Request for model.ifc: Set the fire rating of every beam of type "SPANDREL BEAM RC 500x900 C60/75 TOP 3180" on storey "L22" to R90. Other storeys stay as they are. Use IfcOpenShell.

First a look at what the model holds.

```python
import ifcopenshell
import ifcopenshell.util.element

model = ifcopenshell.open("model.ifc")
print(model.schema)
storey = next(s for s in model.by_type("IfcBuildingStorey") if s.Name == "L22")
beams = [e for e in ifcopenshell.util.element.get_decomposition(storey) if e.is_a("IfcBeam")]
seen = {}
for e in beams:
    element_type = ifcopenshell.util.element.get_type(e)
    key = (element_type.Name if element_type != e and element_type else None, ifcopenshell.util.element.get_pset(e, "Pset_BeamCommon", "FireRating"))
    seen[key] = seen.get(key, 0) + 1
for (name, value), count in sorted(seen.items(), key=str):
    print(count, "x", name, "|", value)
```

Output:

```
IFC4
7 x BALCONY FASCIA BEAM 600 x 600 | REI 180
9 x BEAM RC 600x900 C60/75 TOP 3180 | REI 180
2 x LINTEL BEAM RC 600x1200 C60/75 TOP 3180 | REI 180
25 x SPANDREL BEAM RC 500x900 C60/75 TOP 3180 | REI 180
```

```python
import ifcopenshell
import ifcopenshell.api.pset
import ifcopenshell.util.element

model = ifcopenshell.open("model.ifc")

storey = next(s for s in model.by_type("IfcBuildingStorey") if s.Name == "L22")
beams = [e for e in ifcopenshell.util.element.get_decomposition(storey) if e.is_a("IfcBeam")]

count = 0
for e in beams:
    element_type = ifcopenshell.util.element.get_type(e)
    if element_type in (None, e) or element_type.Name != "SPANDREL BEAM RC 500x900 C60/75 TOP 3180":
        continue
    found = ifcopenshell.util.element.get_pset(e, "Pset_BeamCommon", should_inherit=False)
    if found:
        pset = model.by_id(found["id"])
        if len(ifcopenshell.util.element.get_elements_by_pset(pset)) > 1:
            pset = ifcopenshell.api.pset.unshare_pset(model, products=[e], pset=pset)[0]
    else:
        pset = ifcopenshell.api.pset.add_pset(model, product=e, name="Pset_BeamCommon")
    ifcopenshell.api.pset.edit_pset(model, pset=pset, properties={"FireRating": "R90"})
    count += 1

print(count, "beams updated")

model.write("model_v2.ifc")
```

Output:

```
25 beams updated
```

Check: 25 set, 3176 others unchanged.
